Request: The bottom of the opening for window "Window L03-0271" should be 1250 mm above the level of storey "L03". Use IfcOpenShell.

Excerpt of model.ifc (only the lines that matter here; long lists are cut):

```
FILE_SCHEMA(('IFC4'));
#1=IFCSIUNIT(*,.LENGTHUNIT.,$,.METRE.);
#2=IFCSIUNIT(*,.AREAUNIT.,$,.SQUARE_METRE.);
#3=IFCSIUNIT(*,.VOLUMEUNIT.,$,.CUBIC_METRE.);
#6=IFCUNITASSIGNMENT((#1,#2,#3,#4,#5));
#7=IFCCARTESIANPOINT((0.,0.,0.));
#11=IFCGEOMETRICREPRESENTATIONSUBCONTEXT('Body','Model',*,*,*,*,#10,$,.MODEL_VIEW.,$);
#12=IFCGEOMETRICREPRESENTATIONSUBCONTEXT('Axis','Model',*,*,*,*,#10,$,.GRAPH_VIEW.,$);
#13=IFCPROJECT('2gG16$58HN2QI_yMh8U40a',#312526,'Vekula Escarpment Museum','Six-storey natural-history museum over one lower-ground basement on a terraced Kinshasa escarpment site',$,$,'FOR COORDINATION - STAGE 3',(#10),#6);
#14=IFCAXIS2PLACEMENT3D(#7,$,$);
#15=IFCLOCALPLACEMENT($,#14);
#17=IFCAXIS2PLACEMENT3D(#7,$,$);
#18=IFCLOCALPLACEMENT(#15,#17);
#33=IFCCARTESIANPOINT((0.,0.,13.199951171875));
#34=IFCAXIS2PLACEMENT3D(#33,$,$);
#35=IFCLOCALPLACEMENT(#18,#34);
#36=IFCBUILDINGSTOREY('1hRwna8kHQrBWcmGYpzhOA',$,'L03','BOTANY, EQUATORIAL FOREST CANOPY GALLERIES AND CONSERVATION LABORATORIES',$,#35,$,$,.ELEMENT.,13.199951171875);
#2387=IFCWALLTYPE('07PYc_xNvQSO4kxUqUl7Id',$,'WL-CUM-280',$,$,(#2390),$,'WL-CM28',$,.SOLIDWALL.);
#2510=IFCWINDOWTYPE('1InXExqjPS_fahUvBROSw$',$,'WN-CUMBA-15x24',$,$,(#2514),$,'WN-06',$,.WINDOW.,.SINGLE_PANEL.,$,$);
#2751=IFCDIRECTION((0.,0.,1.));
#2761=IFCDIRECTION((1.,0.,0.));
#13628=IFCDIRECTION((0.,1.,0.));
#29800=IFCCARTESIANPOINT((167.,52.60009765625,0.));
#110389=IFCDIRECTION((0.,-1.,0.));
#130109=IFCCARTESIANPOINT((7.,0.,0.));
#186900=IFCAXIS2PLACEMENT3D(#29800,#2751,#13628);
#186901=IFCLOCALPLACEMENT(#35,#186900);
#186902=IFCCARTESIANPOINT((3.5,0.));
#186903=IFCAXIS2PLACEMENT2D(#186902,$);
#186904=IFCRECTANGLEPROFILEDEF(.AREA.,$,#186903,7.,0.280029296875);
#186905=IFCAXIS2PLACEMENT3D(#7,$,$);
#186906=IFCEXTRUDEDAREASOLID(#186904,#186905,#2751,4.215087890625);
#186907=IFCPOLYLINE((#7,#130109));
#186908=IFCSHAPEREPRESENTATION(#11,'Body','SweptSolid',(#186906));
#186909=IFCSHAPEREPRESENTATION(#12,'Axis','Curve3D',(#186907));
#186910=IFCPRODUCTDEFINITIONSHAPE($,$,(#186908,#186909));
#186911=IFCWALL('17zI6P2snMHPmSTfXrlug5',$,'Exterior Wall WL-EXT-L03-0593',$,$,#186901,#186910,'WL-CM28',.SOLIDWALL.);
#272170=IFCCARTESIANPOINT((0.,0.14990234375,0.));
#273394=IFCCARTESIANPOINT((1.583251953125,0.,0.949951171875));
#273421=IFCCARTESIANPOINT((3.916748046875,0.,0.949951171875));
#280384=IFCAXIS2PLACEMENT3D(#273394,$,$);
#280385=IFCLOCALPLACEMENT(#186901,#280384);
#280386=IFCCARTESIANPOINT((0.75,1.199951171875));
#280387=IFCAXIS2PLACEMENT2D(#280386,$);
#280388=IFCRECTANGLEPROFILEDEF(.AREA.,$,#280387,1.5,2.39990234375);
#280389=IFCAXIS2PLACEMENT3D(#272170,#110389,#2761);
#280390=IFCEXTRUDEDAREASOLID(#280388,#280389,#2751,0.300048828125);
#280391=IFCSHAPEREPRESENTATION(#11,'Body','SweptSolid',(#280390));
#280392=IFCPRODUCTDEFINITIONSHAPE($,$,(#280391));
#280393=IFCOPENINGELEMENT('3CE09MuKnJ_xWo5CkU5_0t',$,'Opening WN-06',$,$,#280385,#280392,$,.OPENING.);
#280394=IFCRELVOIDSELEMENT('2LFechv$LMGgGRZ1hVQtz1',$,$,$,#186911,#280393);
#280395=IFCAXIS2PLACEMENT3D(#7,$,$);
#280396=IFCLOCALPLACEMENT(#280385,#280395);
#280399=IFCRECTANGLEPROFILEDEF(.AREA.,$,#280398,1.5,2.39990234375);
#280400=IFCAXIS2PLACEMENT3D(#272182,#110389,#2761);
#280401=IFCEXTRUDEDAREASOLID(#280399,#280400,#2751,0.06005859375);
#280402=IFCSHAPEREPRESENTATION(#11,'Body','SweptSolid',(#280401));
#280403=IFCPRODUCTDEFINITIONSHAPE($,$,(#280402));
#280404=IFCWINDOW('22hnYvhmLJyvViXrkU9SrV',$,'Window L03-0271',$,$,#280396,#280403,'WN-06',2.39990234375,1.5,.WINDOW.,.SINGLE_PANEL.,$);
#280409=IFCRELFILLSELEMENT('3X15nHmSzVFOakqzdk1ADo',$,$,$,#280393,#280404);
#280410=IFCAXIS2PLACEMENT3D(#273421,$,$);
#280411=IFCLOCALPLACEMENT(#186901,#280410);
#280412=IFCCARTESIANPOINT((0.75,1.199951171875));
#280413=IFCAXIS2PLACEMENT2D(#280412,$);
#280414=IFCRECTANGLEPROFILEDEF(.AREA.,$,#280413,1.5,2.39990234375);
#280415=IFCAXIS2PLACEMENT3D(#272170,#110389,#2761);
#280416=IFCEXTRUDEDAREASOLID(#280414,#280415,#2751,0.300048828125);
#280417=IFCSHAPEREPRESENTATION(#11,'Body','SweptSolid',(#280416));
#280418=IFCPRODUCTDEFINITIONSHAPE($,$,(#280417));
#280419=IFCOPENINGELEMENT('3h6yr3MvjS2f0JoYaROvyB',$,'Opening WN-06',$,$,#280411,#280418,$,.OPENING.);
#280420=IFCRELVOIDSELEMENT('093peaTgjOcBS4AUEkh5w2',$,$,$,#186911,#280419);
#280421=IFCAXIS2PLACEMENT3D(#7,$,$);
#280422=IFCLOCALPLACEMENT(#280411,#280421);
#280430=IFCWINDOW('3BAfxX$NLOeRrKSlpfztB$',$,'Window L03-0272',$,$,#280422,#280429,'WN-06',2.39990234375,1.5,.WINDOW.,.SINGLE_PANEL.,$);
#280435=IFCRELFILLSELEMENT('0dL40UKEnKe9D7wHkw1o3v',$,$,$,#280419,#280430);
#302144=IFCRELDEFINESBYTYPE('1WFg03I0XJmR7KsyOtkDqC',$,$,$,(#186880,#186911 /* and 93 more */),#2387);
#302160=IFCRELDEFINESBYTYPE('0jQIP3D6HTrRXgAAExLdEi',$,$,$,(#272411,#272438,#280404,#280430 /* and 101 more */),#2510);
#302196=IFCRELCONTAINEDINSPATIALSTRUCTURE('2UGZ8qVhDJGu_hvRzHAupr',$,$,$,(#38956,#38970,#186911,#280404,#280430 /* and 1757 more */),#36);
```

```python
import numpy as np
import ifcopenshell
import ifcopenshell.api.geometry
import ifcopenshell.geom
import ifcopenshell.util.element
import ifcopenshell.util.placement
import ifcopenshell.util.shape
import ifcopenshell.util.unit

model = ifcopenshell.open("model.ifc")
unit_scale = ifcopenshell.util.unit.calculate_unit_scale(model)

window = model.by_id(280404)
opening = window.FillsVoids[0].RelatingOpeningElement
storey = ifcopenshell.util.element.get_container(window, ifc_class="IfcBuildingStorey")
level = ifcopenshell.util.placement.get_local_placement(storey.ObjectPlacement)[2, 3]

# The opening's origin need not be at the sill, so measure its lowest point.
shape = ifcopenshell.geom.create_shape(ifcopenshell.geom.settings(), opening)
bottom = ifcopenshell.util.shape.get_shape_bottom_elevation(shape, shape.geometry) / unit_scale
dz = level + 1.25 / unit_scale - bottom

shift = np.array([0.0, 0.0, dz])
# The window is placed relative to its opening, so it follows when the opening moves.
matrix = ifcopenshell.util.placement.get_local_placement(opening.ObjectPlacement)
matrix[:3, 3] += shift
ifcopenshell.api.geometry.edit_object_placement(
    model, product=opening, matrix=matrix, is_si=False, should_transform_children=True
)

print(f"moved by {dz * unit_scale:+.3f} m")

model.write("model-out.ifc")
```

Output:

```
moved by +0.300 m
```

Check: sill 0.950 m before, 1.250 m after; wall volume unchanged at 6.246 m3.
